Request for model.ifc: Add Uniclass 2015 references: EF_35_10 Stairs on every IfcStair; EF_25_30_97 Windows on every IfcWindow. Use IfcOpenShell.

First a look at what the model holds.

```python
import ifcopenshell

model = ifcopenshell.open("model.ifc")
print(model.schema)
print("classifications:", [c.Name for c in model.by_type("IfcClassification")])
for ifc_class in ("IfcDoor", "IfcRoof", "IfcStair", "IfcWall", "IfcWindow"):
    print(ifc_class, len(model.by_type(ifc_class)))
```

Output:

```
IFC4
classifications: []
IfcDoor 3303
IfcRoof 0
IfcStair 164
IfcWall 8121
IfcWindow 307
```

```python
import ifcopenshell
import ifcopenshell.api.classification

model = ifcopenshell.open("model.ifc")

system = ifcopenshell.api.classification.add_classification(model, classification="Uniclass 2015")

codes = {
    "IfcStair": ("EF_35_10", "Stairs"),
    "IfcWindow": ("EF_25_30_97", "Windows"),
}
for ifc_class, (code, name) in codes.items():
    products = model.by_type(ifc_class)
    ifcopenshell.api.classification.add_reference(
        model, products=products, classification=system, identification=code, name=name
    )
    print(code, len(products))

model.write("model-out.ifc")
```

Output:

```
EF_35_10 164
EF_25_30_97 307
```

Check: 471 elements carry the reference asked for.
